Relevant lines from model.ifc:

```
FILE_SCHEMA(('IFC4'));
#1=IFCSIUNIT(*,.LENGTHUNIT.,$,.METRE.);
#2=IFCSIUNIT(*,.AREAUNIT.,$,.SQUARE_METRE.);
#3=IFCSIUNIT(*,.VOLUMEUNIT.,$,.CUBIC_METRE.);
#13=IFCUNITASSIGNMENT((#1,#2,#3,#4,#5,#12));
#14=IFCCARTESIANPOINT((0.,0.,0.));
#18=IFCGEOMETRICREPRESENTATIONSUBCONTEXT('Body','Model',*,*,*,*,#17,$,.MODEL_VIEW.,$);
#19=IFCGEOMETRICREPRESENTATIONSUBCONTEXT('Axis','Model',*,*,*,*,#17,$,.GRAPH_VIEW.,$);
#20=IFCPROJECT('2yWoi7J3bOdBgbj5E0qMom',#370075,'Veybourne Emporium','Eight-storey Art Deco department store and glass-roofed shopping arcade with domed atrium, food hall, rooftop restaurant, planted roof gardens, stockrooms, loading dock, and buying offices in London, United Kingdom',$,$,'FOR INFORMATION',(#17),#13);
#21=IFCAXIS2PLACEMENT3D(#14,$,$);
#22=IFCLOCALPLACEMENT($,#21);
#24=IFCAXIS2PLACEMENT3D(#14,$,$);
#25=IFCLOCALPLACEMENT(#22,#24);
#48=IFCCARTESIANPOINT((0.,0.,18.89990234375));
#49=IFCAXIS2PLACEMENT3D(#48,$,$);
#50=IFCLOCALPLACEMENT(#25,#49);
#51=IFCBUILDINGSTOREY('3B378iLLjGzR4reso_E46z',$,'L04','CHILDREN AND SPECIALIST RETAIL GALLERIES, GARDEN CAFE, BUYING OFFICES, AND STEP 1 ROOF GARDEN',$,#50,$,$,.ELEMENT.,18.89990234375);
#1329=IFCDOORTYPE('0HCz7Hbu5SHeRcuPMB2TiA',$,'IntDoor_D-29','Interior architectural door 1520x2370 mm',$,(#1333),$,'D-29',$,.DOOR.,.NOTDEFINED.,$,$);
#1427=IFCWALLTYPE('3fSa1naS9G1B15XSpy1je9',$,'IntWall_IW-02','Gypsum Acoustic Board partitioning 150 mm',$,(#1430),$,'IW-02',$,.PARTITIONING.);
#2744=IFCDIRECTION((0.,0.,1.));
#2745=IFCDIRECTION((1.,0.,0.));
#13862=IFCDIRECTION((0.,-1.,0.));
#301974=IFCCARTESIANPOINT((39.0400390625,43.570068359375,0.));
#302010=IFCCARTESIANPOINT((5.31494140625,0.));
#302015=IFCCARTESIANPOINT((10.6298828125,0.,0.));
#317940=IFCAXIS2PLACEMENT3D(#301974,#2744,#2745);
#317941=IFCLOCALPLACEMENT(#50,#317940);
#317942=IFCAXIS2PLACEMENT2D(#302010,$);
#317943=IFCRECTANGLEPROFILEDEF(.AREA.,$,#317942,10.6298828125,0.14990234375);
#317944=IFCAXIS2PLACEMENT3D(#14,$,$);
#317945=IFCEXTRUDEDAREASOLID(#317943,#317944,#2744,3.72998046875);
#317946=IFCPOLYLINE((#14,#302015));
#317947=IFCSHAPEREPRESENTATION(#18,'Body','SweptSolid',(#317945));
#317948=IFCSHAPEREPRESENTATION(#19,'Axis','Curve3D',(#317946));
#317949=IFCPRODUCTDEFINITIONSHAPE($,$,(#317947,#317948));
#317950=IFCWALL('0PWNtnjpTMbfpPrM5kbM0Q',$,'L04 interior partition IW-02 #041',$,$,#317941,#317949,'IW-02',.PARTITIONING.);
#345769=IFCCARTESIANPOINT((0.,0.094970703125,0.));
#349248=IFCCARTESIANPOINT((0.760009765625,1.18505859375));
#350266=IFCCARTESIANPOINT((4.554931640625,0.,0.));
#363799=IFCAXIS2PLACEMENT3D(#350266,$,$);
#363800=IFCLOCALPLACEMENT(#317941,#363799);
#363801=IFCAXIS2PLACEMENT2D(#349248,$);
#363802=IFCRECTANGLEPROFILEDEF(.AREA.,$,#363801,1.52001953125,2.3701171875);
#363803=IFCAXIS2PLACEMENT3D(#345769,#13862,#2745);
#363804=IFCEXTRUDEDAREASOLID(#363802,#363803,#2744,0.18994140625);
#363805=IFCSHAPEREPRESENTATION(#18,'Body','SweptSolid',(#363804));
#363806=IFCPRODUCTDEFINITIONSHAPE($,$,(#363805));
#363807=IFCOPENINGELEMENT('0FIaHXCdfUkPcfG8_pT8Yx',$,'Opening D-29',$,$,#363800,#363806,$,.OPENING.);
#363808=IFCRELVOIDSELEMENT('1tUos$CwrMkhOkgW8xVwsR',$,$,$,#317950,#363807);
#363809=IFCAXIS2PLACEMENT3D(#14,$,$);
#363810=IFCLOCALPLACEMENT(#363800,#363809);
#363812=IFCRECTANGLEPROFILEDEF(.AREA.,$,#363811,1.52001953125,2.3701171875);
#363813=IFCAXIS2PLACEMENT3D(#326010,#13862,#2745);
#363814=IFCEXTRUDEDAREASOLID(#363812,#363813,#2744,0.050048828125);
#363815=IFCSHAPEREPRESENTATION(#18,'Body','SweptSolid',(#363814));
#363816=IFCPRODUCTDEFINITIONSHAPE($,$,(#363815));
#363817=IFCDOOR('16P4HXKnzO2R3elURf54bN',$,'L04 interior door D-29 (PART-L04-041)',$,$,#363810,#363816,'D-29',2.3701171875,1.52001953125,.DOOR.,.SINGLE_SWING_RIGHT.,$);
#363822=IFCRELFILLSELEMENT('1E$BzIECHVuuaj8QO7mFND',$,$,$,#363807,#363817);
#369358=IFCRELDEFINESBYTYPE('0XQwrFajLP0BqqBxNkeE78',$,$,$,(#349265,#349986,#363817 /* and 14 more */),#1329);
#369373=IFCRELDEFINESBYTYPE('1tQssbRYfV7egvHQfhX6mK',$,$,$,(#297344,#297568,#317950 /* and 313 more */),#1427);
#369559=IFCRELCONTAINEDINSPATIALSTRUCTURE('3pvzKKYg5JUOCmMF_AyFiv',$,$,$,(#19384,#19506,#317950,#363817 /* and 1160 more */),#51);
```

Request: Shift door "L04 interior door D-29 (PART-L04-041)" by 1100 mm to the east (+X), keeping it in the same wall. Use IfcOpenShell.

```python
import ifcopenshell
import ifcopenshell.api.geometry
import ifcopenshell.util.placement
import ifcopenshell.util.unit

model = ifcopenshell.open("model.ifc")
unit_scale = ifcopenshell.util.unit.calculate_unit_scale(model)

door = model.by_guid("16P4HXKnzO2R3elURf54bN")
opening = door.FillsVoids[0].RelatingOpeningElement
wall = opening.VoidsElements[0].RelatingBuildingElement

wall_matrix = ifcopenshell.util.placement.get_local_placement(wall.ObjectPlacement)
shift = wall_matrix[:3, 0] * 1.1 / unit_scale
before = ifcopenshell.util.placement.get_local_placement(door.ObjectPlacement)[:3, 3].copy()

# The door is placed relative to its opening, so it follows when the opening moves.
matrix = ifcopenshell.util.placement.get_local_placement(opening.ObjectPlacement)
matrix[:3, 3] += shift
ifcopenshell.api.geometry.edit_object_placement(
    model, product=opening, matrix=matrix, is_si=False, should_transform_children=True
)

after = ifcopenshell.util.placement.get_local_placement(door.ObjectPlacement)[:3, 3]
print("door moved by", (after - before).round(3) + 0.0)

model.write("model_rev.ifc")
```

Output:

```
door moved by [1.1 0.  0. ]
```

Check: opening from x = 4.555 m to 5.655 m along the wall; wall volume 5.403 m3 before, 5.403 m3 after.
